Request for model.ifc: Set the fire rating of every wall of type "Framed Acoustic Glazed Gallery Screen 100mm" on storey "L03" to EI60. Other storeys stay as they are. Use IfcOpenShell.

First a look at what the model holds.

```python
import ifcopenshell
import ifcopenshell.util.element

model = ifcopenshell.open("model.ifc")
print(model.schema)
storey = next(s for s in model.by_type("IfcBuildingStorey") if s.Name == "L03")
walls = [e for e in ifcopenshell.util.element.get_decomposition(storey) if e.is_a("IfcWall")]
seen = {}
for e in walls:
    element_type = ifcopenshell.util.element.get_type(e)
    key = (element_type.Name if element_type != e and element_type else None, ifcopenshell.util.element.get_pset(e, "Pset_WallCommon", "FireRating"))
    seen[key] = seen.get(key, 0) + 1
for (name, value), count in sorted(seen.items(), key=str):
    print(count, "x", name, "|", value)
```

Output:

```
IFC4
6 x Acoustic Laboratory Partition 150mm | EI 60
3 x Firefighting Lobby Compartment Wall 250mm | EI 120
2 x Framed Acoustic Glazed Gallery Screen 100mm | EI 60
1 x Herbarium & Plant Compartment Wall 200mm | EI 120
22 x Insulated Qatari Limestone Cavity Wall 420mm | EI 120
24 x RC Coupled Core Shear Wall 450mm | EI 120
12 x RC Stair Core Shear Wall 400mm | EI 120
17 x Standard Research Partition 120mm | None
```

```python
import ifcopenshell
import ifcopenshell.api.pset
import ifcopenshell.util.element

model = ifcopenshell.open("model.ifc")

storey = next(s for s in model.by_type("IfcBuildingStorey") if s.Name == "L03")
walls = [e for e in ifcopenshell.util.element.get_decomposition(storey) if e.is_a("IfcWall")]

count = 0
for e in walls:
    element_type = ifcopenshell.util.element.get_type(e)
    if element_type in (None, e) or element_type.Name != "Framed Acoustic Glazed Gallery Screen 100mm":
        continue
    # add_pset returns the element's existing set when there is one.
    pset = ifcopenshell.api.pset.add_pset(model, product=e, name="Pset_WallCommon")
    ifcopenshell.api.pset.edit_pset(model, pset=pset, properties={"FireRating": "EI60"})
    count += 1

print(count, "walls updated")

model.write("model-out.ifc")
```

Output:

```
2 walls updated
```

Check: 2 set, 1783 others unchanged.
